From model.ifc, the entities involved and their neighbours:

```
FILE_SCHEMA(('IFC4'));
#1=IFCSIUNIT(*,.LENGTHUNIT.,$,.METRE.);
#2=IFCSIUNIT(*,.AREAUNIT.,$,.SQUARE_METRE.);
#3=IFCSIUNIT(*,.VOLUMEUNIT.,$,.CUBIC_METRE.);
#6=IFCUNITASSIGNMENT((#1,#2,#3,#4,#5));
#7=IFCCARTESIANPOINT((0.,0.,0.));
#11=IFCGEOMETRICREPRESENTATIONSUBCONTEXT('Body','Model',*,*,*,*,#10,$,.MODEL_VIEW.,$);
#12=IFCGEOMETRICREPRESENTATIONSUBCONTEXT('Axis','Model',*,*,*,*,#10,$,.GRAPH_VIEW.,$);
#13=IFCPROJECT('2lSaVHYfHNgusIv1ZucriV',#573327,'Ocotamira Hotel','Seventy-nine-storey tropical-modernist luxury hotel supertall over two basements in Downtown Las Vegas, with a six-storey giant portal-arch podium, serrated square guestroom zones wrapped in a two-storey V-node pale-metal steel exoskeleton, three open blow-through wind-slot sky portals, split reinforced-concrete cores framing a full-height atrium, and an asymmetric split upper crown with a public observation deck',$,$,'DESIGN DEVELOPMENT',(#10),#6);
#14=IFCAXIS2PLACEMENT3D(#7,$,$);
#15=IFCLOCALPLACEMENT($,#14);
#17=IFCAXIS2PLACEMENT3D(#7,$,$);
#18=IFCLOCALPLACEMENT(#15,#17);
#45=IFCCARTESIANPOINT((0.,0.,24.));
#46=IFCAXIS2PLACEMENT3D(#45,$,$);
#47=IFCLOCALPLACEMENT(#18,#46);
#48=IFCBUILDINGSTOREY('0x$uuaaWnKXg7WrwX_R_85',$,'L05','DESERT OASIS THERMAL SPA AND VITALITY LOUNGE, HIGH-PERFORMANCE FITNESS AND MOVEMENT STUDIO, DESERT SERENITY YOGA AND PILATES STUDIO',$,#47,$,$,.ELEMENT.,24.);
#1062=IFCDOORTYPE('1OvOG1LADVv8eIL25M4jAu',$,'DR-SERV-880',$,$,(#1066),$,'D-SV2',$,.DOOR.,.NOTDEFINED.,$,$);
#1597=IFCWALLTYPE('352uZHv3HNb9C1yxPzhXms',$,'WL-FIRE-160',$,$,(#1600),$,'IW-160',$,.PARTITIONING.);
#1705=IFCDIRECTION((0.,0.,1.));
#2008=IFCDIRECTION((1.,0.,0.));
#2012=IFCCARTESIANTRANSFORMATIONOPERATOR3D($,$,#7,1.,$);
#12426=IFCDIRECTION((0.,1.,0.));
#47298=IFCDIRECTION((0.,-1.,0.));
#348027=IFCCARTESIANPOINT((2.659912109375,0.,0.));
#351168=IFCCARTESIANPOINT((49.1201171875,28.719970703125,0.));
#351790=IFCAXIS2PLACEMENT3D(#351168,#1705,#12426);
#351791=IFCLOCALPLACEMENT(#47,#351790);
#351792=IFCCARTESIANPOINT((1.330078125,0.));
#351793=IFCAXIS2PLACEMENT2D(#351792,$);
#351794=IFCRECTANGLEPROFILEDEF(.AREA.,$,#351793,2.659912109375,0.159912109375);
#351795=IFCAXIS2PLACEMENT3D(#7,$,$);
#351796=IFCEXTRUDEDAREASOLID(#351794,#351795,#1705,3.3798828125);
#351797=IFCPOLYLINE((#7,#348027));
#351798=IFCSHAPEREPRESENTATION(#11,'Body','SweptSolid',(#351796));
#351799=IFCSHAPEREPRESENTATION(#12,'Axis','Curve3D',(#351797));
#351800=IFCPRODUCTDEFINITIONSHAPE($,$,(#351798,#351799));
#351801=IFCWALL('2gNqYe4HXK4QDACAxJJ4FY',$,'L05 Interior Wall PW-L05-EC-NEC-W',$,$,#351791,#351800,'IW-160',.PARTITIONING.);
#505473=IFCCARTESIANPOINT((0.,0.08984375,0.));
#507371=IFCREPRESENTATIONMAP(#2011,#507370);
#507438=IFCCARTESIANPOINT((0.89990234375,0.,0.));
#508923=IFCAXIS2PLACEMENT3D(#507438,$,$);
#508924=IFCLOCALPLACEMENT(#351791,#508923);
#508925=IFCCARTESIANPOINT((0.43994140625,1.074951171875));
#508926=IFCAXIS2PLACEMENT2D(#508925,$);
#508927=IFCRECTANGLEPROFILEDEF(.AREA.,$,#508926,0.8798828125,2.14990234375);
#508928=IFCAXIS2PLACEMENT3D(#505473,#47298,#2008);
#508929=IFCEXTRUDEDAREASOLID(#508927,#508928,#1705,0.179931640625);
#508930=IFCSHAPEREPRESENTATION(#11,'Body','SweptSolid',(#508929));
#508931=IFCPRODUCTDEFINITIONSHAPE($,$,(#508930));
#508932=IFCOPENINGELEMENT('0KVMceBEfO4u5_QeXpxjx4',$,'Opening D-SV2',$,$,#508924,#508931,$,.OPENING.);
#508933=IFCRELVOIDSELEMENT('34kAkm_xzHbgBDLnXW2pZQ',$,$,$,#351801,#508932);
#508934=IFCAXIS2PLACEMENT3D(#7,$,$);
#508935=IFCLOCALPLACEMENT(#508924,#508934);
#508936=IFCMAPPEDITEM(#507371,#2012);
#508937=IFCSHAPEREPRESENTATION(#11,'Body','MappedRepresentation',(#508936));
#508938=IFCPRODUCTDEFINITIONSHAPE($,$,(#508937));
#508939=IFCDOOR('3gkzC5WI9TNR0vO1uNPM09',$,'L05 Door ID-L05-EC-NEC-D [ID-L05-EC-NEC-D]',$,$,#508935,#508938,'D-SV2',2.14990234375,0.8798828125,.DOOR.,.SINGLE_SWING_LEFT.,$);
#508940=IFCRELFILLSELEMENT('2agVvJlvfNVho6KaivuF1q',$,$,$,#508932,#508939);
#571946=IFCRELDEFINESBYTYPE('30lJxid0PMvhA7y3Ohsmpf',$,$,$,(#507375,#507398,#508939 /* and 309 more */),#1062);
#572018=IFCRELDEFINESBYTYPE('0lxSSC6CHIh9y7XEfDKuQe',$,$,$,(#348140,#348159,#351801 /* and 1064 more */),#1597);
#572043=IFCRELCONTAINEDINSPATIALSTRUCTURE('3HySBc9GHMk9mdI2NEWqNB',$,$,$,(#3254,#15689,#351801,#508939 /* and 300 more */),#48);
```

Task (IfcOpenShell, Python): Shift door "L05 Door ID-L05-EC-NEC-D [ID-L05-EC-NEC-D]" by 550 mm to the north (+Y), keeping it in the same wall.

```python
import ifcopenshell
import ifcopenshell.api.geometry
import ifcopenshell.util.placement

model = ifcopenshell.open("model.ifc")

door = model.by_guid("3gkzC5WI9TNR0vO1uNPM09")
opening = door.FillsVoids[0].RelatingOpeningElement
wall = opening.VoidsElements[0].RelatingBuildingElement

wall_matrix = ifcopenshell.util.placement.get_local_placement(wall.ObjectPlacement)
shift = wall_matrix[:3, 0] * 0.55
before = ifcopenshell.util.placement.get_local_placement(door.ObjectPlacement)[:3, 3].copy()

# The door is placed relative to its opening, so it follows when the opening moves.
matrix = ifcopenshell.util.placement.get_local_placement(opening.ObjectPlacement)
matrix[:3, 3] += shift
ifcopenshell.api.geometry.edit_object_placement(
    model, product=opening, matrix=matrix, is_si=False, should_transform_children=True
)

after = ifcopenshell.util.placement.get_local_placement(door.ObjectPlacement)[:3, 3]
print("door moved by", (after - before).round(3) + 0.0)

model.write("model_v2.ifc")
```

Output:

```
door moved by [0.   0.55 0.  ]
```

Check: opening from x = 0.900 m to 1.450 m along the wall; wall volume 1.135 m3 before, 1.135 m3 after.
